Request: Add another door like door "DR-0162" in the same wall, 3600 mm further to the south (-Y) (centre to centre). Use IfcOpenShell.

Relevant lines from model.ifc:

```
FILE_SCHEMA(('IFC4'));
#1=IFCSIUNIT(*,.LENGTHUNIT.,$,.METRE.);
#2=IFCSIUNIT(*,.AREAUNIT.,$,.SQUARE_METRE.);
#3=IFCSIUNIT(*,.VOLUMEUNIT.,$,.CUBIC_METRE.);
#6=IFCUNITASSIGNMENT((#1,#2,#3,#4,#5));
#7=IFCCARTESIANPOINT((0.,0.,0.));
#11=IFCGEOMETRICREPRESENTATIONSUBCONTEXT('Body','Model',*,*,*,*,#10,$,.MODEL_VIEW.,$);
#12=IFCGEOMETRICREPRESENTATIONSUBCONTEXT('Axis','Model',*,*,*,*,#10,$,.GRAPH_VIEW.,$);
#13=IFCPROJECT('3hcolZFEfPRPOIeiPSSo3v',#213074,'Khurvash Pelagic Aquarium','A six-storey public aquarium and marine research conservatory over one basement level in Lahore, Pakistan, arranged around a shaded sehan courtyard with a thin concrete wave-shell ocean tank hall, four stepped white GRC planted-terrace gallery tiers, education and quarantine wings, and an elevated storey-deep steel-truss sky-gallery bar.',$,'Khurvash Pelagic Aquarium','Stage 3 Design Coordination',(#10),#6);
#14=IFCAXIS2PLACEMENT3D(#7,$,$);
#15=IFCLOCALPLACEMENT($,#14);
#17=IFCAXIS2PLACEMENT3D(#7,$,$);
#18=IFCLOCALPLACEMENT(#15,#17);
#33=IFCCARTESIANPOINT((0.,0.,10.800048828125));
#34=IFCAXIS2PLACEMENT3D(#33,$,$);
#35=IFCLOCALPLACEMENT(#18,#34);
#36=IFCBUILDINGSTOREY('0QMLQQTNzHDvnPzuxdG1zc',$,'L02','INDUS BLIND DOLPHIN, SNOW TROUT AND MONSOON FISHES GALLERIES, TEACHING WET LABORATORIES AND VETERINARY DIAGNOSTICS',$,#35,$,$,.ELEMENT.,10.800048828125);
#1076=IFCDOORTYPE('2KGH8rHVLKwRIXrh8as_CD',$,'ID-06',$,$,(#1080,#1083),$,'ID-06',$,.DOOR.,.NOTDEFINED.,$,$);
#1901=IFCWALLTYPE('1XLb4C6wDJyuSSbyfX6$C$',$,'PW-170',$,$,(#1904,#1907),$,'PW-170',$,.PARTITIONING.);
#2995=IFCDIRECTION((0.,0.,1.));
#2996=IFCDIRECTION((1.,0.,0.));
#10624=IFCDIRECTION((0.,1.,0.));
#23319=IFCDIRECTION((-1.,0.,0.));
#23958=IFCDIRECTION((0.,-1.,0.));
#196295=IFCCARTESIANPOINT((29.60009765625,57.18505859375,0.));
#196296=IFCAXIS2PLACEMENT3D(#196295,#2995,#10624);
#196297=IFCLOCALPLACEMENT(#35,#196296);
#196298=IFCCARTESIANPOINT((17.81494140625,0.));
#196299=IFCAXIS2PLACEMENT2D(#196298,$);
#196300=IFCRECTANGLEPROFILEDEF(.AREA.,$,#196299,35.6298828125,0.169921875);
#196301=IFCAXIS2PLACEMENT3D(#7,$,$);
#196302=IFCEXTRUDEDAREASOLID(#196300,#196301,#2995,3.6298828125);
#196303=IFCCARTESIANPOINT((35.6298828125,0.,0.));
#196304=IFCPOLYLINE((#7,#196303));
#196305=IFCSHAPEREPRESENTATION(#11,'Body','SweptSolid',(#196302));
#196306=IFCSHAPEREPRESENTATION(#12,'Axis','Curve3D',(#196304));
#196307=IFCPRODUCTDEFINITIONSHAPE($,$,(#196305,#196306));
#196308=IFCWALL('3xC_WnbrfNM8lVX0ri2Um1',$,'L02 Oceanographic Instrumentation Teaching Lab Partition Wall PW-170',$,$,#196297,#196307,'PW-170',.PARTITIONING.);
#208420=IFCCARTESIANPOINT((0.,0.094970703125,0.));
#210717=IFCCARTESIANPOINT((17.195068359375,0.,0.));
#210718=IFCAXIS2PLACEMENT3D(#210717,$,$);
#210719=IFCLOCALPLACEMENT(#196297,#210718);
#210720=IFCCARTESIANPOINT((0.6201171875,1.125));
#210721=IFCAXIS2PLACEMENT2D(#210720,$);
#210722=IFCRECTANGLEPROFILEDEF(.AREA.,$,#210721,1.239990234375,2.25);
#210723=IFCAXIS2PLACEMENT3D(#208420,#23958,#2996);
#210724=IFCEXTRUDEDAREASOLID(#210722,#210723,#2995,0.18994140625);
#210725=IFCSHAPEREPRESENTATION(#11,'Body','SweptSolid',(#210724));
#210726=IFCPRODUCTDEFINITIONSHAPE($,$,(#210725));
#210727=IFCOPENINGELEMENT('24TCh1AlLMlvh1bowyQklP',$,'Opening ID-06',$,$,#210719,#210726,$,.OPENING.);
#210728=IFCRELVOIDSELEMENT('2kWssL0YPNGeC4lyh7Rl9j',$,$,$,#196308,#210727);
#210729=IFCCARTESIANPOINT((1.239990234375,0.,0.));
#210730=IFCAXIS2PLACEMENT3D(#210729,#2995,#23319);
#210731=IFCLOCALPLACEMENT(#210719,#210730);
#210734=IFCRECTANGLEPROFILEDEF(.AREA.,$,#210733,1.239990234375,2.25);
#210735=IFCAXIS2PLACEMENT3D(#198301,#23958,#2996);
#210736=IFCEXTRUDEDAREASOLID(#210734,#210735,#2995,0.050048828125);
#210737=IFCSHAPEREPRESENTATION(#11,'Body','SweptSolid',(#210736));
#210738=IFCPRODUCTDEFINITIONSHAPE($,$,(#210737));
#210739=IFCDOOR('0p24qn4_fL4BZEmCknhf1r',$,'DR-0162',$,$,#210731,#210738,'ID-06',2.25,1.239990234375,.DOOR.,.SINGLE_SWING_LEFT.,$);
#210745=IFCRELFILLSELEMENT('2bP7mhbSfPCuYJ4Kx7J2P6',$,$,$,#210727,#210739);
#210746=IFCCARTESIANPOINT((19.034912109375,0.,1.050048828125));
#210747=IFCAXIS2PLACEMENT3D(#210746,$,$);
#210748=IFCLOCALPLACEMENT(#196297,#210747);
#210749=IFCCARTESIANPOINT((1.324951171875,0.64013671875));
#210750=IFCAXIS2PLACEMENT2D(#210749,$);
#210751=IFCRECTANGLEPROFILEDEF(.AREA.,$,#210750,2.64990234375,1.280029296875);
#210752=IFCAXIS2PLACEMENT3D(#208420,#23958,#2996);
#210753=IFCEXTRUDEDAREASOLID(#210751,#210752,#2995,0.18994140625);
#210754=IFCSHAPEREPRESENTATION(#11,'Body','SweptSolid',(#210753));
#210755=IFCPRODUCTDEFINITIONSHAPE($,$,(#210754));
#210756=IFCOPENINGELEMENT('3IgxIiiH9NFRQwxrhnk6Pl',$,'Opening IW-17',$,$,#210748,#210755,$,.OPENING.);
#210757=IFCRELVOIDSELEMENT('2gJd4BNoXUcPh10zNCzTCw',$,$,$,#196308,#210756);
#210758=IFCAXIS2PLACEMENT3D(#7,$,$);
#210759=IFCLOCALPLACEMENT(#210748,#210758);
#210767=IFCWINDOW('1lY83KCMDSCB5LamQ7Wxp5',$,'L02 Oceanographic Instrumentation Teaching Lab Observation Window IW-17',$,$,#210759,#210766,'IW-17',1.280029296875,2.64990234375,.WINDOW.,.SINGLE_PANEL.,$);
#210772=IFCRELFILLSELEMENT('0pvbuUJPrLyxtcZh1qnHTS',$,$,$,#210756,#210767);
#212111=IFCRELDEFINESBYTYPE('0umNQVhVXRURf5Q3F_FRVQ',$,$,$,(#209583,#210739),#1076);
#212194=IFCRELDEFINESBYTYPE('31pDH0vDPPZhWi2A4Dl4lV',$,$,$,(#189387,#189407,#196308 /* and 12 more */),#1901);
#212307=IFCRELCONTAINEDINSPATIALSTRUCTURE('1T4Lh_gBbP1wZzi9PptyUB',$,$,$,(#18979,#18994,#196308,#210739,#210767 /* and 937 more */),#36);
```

```python
import ifcopenshell
import ifcopenshell.api.feature
import ifcopenshell.api.geometry
import ifcopenshell.api.root
import ifcopenshell.geom
import ifcopenshell.util.element
import ifcopenshell.util.placement
import ifcopenshell.util.shape
import ifcopenshell.util.unit

model = ifcopenshell.open("model.ifc")
unit_scale = ifcopenshell.util.unit.calculate_unit_scale(model)
settings = ifcopenshell.geom.settings()


def volume(element):
    """Net volume in cubic metres, openings subtracted."""
    shape = ifcopenshell.geom.create_shape(settings, element)
    return ifcopenshell.util.shape.get_volume(shape.geometry)


door = model.by_guid("0p24qn4_fL4BZEmCknhf1r")
opening = door.FillsVoids[0].RelatingOpeningElement
wall = opening.VoidsElements[0].RelatingBuildingElement
before = volume(wall)
shift = ifcopenshell.util.placement.get_local_placement(wall.ObjectPlacement)[:3, 0] * -3.6 / unit_scale

# copy_class copies the void relationship, type, container and properties, but no geometry.
new_opening = ifcopenshell.api.root.copy_class(model, product=opening)
new_opening.Representation = ifcopenshell.util.element.copy_deep(
    model, opening.Representation, exclude=["IfcGeometricRepresentationContext", "IfcRepresentationMap"]
)
new_door = ifcopenshell.api.root.copy_class(model, product=door)
new_door.Representation = ifcopenshell.util.element.copy_deep(
    model, door.Representation, exclude=["IfcGeometricRepresentationContext", "IfcRepresentationMap"]
)
new_door.Tag = None
ifcopenshell.api.feature.add_filling(model, opening=new_opening, element=new_door)

for old, new in ((opening, new_opening), (door, new_door)):
    matrix = ifcopenshell.util.placement.get_local_placement(old.ObjectPlacement)
    matrix[:3, 3] += shift
    ifcopenshell.api.geometry.edit_object_placement(model, product=new, matrix=matrix, is_si=False)

after = volume(wall)

print(f"wall volume {before:.3f} -> {after:.3f} m3")

model.write("model_rev.ifc")
```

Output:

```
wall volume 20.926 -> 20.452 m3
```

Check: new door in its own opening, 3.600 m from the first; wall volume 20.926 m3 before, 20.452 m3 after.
